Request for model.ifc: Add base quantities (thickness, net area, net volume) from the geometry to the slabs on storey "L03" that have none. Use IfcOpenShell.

First a look at what the model holds.

```python
import ifcopenshell
import ifcopenshell.util.element
import ifcopenshell.util.unit

model = ifcopenshell.open("model.ifc")
print(model.schema)
for unit_type in ("LENGTHUNIT", "AREAUNIT", "VOLUMEUNIT"):
    print(unit_type, ifcopenshell.util.unit.calculate_unit_scale(model, unit_type))
storey = next(s for s in model.by_type("IfcBuildingStorey") if s.Name == "L03")
slabs = [e for e in ifcopenshell.util.element.get_decomposition(storey) if e.is_a("IfcSlab")]
for e in sorted(slabs, key=lambda e: e.id()):
    print(e.id(), e.is_a(), e.Name, list(ifcopenshell.util.element.get_psets(e, qtos_only=True)), sep=" | ")
```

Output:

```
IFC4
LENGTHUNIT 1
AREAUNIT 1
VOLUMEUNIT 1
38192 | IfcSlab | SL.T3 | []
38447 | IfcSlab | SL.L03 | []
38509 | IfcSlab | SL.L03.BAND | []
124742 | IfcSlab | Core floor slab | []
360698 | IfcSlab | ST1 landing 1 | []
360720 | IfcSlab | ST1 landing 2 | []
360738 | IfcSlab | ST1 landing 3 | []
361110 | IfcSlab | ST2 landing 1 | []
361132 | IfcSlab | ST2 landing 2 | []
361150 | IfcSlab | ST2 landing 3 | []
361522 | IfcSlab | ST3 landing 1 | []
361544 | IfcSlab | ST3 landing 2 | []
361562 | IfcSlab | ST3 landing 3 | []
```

```python
import ifcopenshell
import ifcopenshell.api.pset
import ifcopenshell.geom
import ifcopenshell.util.element
import ifcopenshell.util.shape
import ifcopenshell.util.unit

model = ifcopenshell.open("model.ifc")
unit_scale = ifcopenshell.util.unit.calculate_unit_scale(model)
area_scale = ifcopenshell.util.unit.calculate_unit_scale(model, "AREAUNIT")
volume_scale = ifcopenshell.util.unit.calculate_unit_scale(model, "VOLUMEUNIT")
settings = ifcopenshell.geom.settings()

storey = next(s for s in model.by_type("IfcBuildingStorey") if s.Name == "L03")
slabs = [e for e in ifcopenshell.util.element.get_decomposition(storey) if e.is_a("IfcSlab")]

for e in sorted(slabs, key=lambda e: e.id()):
    if ifcopenshell.util.element.get_psets(e, qtos_only=True, should_inherit=False):
        continue
    # Geometry comes back in metres, in the element's own axes.
    shape = ifcopenshell.geom.create_shape(settings, e)
    values = {
        "Width": ifcopenshell.util.shape.get_z(shape.geometry) / unit_scale,
        "NetArea": ifcopenshell.util.shape.get_footprint_area(shape.geometry) / area_scale,
        "NetVolume": ifcopenshell.util.shape.get_volume(shape.geometry) / volume_scale,
    }
    qto = ifcopenshell.api.pset.add_qto(model, product=e, name="Qto_SlabBaseQuantities")
    ifcopenshell.api.pset.edit_qto(model, qto=qto, properties=values)
    print(e.id(), {k: round(v, 3) for k, v in values.items()})

model.write("model-out.ifc")
```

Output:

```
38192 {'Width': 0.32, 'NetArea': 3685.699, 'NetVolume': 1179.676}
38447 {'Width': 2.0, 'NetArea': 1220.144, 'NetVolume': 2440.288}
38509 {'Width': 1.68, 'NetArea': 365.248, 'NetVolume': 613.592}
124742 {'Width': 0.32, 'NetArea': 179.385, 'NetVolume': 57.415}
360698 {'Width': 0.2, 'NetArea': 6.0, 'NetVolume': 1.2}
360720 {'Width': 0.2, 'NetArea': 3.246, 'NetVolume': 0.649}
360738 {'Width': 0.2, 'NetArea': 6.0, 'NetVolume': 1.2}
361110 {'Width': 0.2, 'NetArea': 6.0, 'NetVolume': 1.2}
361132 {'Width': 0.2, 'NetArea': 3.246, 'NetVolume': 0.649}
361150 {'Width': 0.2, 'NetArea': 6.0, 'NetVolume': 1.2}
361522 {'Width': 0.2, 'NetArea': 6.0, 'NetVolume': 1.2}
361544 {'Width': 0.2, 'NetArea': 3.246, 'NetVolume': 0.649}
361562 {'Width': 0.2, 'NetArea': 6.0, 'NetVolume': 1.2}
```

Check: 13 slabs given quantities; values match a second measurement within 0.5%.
